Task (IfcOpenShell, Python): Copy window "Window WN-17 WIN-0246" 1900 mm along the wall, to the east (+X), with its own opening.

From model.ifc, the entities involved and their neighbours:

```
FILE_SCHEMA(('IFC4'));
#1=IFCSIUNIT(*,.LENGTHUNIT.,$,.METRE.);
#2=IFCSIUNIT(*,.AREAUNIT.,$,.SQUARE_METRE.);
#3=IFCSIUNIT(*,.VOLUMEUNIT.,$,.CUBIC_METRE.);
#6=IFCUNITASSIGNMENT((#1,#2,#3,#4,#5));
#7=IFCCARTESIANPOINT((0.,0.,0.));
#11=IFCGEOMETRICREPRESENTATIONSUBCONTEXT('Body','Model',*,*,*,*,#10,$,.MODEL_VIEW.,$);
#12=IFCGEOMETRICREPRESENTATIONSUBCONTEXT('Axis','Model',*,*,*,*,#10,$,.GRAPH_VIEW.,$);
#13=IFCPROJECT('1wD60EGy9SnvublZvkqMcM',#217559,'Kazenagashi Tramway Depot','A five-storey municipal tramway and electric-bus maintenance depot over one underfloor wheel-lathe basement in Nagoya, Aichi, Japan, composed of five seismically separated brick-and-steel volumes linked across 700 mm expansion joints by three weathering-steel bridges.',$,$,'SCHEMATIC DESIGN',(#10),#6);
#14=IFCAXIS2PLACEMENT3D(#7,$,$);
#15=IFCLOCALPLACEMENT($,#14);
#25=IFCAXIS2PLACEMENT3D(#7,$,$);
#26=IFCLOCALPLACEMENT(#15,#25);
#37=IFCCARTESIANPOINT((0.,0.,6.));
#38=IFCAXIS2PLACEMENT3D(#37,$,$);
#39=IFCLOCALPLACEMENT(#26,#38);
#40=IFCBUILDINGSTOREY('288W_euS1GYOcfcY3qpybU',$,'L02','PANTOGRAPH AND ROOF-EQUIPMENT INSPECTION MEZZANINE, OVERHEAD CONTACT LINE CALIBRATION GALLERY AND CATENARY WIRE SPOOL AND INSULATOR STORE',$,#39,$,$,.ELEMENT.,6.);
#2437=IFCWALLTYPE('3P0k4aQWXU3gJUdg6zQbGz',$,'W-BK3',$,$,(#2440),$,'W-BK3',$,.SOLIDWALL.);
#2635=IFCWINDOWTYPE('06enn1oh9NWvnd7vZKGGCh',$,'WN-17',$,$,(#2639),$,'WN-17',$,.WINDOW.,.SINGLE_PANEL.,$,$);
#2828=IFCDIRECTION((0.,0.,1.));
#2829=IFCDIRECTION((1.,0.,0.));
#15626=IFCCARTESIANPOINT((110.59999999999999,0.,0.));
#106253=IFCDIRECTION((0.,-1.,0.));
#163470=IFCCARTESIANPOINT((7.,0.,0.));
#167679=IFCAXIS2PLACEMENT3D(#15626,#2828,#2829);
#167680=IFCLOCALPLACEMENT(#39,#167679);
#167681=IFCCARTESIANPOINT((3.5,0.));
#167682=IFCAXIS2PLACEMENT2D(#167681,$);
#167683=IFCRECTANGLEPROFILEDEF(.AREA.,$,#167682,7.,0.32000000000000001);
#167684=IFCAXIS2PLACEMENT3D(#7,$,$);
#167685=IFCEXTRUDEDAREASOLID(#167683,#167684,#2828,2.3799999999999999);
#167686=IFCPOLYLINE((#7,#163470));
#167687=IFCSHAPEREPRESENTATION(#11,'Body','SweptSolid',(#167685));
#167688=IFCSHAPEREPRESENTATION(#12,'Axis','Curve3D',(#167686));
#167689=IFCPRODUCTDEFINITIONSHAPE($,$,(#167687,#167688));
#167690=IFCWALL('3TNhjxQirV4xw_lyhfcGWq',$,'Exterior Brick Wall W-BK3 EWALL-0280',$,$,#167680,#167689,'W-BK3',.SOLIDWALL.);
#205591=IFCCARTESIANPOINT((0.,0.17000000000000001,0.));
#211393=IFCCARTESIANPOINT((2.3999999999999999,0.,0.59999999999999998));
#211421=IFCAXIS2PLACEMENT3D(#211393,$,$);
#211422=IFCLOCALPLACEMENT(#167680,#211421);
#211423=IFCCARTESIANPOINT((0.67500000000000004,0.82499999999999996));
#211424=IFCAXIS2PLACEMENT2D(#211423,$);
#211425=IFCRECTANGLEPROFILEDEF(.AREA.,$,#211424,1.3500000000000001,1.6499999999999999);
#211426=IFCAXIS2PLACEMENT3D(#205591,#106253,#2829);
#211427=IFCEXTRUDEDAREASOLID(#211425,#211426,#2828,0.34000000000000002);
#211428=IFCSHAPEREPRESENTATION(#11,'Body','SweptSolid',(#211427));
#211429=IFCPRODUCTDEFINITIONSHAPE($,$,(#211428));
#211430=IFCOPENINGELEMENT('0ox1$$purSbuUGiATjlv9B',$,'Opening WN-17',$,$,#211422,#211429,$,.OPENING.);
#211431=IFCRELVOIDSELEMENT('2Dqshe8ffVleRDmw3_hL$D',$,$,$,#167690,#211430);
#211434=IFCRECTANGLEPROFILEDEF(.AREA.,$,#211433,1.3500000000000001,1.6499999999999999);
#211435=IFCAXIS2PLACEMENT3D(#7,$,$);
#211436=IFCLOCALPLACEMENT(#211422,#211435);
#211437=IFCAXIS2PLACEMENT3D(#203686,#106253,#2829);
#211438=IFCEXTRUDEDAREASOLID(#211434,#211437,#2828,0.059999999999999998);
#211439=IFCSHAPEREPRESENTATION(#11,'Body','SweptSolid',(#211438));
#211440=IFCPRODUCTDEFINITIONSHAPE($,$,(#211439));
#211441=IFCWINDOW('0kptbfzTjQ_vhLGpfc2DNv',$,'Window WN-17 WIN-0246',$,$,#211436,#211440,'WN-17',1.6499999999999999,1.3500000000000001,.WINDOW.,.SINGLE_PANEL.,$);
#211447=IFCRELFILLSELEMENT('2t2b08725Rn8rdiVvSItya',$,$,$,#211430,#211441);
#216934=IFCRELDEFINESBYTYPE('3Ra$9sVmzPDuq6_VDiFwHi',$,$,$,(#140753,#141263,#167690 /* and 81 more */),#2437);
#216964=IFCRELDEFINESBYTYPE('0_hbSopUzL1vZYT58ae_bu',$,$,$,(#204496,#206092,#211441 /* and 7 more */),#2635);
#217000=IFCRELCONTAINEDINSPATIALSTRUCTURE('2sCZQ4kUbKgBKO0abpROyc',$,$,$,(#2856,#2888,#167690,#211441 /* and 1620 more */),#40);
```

```python
import ifcopenshell
import ifcopenshell.api.feature
import ifcopenshell.api.geometry
import ifcopenshell.api.root
import ifcopenshell.geom
import ifcopenshell.util.element
import ifcopenshell.util.placement
import ifcopenshell.util.shape

model = ifcopenshell.open("model.ifc")
settings = ifcopenshell.geom.settings()


def volume(element):
    """Net volume in cubic metres, openings subtracted."""
    shape = ifcopenshell.geom.create_shape(settings, element)
    return ifcopenshell.util.shape.get_volume(shape.geometry)


window = model.by_guid("0kptbfzTjQ_vhLGpfc2DNv")
opening = window.FillsVoids[0].RelatingOpeningElement
wall = opening.VoidsElements[0].RelatingBuildingElement
before = volume(wall)
shift = ifcopenshell.util.placement.get_local_placement(wall.ObjectPlacement)[:3, 0] * 1.9

# copy_class copies the void relationship, type, container and properties, but no geometry.
new_opening = ifcopenshell.api.root.copy_class(model, product=opening)
new_opening.Representation = ifcopenshell.util.element.copy_deep(
    model, opening.Representation, exclude=["IfcGeometricRepresentationContext", "IfcRepresentationMap"]
)
new_window = ifcopenshell.api.root.copy_class(model, product=window)
new_window.Representation = ifcopenshell.util.element.copy_deep(
    model, window.Representation, exclude=["IfcGeometricRepresentationContext", "IfcRepresentationMap"]
)
new_window.Tag = None
ifcopenshell.api.feature.add_filling(model, opening=new_opening, element=new_window)

for old, new in ((opening, new_opening), (window, new_window)):
    matrix = ifcopenshell.util.placement.get_local_placement(old.ObjectPlacement)
    matrix[:3, 3] += shift
    ifcopenshell.api.geometry.edit_object_placement(model, product=new, matrix=matrix, is_si=False)

after = volume(wall)

print(f"wall volume {before:.3f} -> {after:.3f} m3")

model.write("model_rev.ifc")
```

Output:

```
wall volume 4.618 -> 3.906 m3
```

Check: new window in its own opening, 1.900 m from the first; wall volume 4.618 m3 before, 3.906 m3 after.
